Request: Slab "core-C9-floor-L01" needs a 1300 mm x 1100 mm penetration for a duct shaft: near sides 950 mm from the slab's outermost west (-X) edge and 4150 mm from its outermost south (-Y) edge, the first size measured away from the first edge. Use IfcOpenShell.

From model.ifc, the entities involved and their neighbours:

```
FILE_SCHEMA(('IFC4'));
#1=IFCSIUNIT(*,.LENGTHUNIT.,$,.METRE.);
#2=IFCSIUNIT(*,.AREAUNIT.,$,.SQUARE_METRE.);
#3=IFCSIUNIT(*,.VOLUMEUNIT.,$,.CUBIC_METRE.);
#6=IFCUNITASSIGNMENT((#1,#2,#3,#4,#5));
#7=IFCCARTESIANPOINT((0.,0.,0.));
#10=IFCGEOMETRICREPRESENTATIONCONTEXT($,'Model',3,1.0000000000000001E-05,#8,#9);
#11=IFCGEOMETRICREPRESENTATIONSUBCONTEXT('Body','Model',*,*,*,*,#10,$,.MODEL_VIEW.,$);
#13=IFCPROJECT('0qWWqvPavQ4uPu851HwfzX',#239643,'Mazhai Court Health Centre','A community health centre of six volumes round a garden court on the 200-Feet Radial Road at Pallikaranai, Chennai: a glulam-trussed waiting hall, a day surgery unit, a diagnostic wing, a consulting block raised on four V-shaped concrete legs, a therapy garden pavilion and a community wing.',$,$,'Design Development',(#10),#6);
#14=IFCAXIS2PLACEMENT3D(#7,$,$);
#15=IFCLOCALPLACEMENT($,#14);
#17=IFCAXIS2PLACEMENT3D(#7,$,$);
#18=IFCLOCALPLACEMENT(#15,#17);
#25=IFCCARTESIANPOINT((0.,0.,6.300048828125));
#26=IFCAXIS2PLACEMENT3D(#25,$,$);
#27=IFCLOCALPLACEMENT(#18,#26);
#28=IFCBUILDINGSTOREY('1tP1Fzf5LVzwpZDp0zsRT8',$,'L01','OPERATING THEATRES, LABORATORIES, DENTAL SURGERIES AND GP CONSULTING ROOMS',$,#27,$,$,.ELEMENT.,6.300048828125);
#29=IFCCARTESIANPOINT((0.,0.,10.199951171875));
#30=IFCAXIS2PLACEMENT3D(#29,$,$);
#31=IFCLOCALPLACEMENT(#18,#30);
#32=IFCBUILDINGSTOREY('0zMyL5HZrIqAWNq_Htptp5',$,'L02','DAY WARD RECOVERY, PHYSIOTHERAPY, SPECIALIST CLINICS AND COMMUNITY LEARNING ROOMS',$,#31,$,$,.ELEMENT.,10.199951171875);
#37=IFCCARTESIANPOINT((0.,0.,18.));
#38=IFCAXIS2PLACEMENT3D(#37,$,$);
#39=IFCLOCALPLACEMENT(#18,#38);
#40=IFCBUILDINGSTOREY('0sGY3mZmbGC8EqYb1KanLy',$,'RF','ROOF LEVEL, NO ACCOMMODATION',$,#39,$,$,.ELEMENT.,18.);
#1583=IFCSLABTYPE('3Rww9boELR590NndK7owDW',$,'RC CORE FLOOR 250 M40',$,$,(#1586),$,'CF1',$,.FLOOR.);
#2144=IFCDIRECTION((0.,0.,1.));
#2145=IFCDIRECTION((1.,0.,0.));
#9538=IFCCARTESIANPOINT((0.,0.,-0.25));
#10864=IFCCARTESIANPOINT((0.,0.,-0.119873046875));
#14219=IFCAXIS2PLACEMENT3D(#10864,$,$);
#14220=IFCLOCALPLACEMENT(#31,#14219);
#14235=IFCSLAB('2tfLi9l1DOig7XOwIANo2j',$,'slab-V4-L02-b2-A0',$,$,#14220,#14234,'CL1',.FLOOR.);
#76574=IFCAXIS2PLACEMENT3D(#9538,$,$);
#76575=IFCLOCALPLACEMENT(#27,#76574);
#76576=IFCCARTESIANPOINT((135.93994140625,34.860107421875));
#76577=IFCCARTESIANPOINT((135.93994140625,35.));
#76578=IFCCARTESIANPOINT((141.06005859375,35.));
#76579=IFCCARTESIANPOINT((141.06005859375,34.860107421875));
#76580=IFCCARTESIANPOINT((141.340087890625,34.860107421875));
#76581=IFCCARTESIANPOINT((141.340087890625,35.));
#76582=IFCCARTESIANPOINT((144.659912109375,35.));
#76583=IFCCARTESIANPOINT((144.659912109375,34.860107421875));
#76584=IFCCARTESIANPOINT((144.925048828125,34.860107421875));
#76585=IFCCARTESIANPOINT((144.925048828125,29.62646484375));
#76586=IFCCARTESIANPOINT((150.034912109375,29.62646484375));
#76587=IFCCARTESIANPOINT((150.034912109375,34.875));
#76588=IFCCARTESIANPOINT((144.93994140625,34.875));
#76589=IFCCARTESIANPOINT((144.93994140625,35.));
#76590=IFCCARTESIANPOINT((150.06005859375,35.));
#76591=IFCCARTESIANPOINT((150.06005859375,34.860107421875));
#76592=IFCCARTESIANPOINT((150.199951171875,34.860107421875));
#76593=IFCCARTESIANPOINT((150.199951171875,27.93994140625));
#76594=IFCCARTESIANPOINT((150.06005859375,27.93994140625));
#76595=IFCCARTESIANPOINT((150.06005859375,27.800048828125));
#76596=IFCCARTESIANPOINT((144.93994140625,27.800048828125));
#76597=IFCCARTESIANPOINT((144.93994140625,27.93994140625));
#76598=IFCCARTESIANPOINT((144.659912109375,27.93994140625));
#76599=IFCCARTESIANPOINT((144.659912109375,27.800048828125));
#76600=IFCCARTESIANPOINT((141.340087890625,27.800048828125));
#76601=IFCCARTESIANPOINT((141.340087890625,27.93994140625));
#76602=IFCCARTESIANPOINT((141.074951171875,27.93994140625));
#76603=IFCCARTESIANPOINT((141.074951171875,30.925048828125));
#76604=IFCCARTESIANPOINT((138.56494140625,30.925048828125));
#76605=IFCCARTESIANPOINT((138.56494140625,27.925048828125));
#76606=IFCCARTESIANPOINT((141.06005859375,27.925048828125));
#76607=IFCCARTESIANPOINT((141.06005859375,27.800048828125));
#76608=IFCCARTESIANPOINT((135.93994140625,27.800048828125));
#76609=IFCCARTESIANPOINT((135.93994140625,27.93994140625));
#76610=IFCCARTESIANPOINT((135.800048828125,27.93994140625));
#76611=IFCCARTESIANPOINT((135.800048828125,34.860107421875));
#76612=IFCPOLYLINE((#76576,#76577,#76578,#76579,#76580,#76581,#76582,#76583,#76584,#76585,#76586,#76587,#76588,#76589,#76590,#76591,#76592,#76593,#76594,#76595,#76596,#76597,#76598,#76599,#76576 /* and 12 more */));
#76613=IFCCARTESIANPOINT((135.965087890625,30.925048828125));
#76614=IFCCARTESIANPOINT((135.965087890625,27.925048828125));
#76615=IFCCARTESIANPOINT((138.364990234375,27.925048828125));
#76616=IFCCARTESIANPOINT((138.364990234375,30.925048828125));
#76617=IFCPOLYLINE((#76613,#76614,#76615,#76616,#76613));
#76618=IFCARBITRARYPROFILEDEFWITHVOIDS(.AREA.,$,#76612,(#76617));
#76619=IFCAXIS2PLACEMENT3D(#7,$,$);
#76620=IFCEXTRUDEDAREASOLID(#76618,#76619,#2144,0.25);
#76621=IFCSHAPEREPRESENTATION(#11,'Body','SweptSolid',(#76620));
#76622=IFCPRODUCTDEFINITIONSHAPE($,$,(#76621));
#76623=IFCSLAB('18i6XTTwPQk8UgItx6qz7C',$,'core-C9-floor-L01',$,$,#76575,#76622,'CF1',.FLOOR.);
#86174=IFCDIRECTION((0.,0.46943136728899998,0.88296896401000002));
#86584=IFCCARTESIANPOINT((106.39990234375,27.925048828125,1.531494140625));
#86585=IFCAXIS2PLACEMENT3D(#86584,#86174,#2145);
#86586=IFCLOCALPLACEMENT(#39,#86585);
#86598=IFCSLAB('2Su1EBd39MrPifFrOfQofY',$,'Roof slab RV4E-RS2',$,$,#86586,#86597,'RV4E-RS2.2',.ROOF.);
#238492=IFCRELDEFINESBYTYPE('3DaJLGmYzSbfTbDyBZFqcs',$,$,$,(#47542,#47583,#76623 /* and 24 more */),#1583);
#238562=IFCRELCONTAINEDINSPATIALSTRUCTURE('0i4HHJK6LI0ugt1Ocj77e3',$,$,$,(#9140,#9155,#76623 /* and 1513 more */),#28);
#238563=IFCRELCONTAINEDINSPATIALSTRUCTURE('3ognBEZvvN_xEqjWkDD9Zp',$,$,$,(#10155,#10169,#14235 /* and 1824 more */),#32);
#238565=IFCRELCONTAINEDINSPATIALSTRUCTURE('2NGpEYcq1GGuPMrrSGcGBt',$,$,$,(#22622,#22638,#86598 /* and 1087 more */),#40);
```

```python
import numpy as np
import ifcopenshell
import ifcopenshell.api.feature
import ifcopenshell.api.geometry
import ifcopenshell.api.root
import ifcopenshell.geom
import ifcopenshell.util.placement
import ifcopenshell.util.representation
import ifcopenshell.util.shape
import ifcopenshell.util.unit

model = ifcopenshell.open("model.ifc")
unit_scale = ifcopenshell.util.unit.calculate_unit_scale(model)
settings = ifcopenshell.geom.settings()


def volume(element):
    """Net volume in cubic metres, openings subtracted."""
    shape = ifcopenshell.geom.create_shape(settings, element)
    return ifcopenshell.util.shape.get_volume(shape.geometry)


slab = model.by_guid("18i6XTTwPQk8UgItx6qz7C")
before = volume(slab)

# Extent in the slab's own axes, in metres. The edges named are its -X and -Y sides.
slab_shape = ifcopenshell.geom.create_shape(settings, slab)
vertices = ifcopenshell.util.shape.get_vertices(slab_shape.geometry)
x_min, y_min, bottom = vertices.min(axis=0)
top = vertices[:, 2].max()

opening = ifcopenshell.api.root.create_entity(model, ifc_class="IfcOpeningElement", name="Duct shaft opening", predefined_type="OPENING")
context = ifcopenshell.util.representation.get_context(model, "Model", "Body", "MODEL_VIEW")
width, depth = 1.3, 1.1
outline = [(0.0, 0.0), (width, 0.0), (width, depth), (0.0, depth), (0.0, 0.0)]
# Overshoot both faces by 50 mm so the cut is clean.
shape = ifcopenshell.api.geometry.add_slab_representation(
    model, context=context, depth=top - bottom + 0.1, polyline=outline
)
ifcopenshell.api.geometry.assign_representation(model, product=opening, representation=shape)

matrix = ifcopenshell.util.placement.get_local_placement(slab.ObjectPlacement)
matrix[:, 3] = matrix @ np.append(np.array([x_min + 0.95, y_min + 4.15, bottom - 0.05]) / unit_scale, 1.0)
ifcopenshell.api.geometry.edit_object_placement(model, product=opening, matrix=matrix, is_si=False)
ifcopenshell.api.feature.add_feature(model, feature=opening, element=slab)

after = volume(slab)

print(f"slab volume {before:.3f} -> {after:.3f} m3")

model.write("model_rev.ifc")
```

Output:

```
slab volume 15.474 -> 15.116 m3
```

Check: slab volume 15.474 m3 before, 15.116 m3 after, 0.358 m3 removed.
